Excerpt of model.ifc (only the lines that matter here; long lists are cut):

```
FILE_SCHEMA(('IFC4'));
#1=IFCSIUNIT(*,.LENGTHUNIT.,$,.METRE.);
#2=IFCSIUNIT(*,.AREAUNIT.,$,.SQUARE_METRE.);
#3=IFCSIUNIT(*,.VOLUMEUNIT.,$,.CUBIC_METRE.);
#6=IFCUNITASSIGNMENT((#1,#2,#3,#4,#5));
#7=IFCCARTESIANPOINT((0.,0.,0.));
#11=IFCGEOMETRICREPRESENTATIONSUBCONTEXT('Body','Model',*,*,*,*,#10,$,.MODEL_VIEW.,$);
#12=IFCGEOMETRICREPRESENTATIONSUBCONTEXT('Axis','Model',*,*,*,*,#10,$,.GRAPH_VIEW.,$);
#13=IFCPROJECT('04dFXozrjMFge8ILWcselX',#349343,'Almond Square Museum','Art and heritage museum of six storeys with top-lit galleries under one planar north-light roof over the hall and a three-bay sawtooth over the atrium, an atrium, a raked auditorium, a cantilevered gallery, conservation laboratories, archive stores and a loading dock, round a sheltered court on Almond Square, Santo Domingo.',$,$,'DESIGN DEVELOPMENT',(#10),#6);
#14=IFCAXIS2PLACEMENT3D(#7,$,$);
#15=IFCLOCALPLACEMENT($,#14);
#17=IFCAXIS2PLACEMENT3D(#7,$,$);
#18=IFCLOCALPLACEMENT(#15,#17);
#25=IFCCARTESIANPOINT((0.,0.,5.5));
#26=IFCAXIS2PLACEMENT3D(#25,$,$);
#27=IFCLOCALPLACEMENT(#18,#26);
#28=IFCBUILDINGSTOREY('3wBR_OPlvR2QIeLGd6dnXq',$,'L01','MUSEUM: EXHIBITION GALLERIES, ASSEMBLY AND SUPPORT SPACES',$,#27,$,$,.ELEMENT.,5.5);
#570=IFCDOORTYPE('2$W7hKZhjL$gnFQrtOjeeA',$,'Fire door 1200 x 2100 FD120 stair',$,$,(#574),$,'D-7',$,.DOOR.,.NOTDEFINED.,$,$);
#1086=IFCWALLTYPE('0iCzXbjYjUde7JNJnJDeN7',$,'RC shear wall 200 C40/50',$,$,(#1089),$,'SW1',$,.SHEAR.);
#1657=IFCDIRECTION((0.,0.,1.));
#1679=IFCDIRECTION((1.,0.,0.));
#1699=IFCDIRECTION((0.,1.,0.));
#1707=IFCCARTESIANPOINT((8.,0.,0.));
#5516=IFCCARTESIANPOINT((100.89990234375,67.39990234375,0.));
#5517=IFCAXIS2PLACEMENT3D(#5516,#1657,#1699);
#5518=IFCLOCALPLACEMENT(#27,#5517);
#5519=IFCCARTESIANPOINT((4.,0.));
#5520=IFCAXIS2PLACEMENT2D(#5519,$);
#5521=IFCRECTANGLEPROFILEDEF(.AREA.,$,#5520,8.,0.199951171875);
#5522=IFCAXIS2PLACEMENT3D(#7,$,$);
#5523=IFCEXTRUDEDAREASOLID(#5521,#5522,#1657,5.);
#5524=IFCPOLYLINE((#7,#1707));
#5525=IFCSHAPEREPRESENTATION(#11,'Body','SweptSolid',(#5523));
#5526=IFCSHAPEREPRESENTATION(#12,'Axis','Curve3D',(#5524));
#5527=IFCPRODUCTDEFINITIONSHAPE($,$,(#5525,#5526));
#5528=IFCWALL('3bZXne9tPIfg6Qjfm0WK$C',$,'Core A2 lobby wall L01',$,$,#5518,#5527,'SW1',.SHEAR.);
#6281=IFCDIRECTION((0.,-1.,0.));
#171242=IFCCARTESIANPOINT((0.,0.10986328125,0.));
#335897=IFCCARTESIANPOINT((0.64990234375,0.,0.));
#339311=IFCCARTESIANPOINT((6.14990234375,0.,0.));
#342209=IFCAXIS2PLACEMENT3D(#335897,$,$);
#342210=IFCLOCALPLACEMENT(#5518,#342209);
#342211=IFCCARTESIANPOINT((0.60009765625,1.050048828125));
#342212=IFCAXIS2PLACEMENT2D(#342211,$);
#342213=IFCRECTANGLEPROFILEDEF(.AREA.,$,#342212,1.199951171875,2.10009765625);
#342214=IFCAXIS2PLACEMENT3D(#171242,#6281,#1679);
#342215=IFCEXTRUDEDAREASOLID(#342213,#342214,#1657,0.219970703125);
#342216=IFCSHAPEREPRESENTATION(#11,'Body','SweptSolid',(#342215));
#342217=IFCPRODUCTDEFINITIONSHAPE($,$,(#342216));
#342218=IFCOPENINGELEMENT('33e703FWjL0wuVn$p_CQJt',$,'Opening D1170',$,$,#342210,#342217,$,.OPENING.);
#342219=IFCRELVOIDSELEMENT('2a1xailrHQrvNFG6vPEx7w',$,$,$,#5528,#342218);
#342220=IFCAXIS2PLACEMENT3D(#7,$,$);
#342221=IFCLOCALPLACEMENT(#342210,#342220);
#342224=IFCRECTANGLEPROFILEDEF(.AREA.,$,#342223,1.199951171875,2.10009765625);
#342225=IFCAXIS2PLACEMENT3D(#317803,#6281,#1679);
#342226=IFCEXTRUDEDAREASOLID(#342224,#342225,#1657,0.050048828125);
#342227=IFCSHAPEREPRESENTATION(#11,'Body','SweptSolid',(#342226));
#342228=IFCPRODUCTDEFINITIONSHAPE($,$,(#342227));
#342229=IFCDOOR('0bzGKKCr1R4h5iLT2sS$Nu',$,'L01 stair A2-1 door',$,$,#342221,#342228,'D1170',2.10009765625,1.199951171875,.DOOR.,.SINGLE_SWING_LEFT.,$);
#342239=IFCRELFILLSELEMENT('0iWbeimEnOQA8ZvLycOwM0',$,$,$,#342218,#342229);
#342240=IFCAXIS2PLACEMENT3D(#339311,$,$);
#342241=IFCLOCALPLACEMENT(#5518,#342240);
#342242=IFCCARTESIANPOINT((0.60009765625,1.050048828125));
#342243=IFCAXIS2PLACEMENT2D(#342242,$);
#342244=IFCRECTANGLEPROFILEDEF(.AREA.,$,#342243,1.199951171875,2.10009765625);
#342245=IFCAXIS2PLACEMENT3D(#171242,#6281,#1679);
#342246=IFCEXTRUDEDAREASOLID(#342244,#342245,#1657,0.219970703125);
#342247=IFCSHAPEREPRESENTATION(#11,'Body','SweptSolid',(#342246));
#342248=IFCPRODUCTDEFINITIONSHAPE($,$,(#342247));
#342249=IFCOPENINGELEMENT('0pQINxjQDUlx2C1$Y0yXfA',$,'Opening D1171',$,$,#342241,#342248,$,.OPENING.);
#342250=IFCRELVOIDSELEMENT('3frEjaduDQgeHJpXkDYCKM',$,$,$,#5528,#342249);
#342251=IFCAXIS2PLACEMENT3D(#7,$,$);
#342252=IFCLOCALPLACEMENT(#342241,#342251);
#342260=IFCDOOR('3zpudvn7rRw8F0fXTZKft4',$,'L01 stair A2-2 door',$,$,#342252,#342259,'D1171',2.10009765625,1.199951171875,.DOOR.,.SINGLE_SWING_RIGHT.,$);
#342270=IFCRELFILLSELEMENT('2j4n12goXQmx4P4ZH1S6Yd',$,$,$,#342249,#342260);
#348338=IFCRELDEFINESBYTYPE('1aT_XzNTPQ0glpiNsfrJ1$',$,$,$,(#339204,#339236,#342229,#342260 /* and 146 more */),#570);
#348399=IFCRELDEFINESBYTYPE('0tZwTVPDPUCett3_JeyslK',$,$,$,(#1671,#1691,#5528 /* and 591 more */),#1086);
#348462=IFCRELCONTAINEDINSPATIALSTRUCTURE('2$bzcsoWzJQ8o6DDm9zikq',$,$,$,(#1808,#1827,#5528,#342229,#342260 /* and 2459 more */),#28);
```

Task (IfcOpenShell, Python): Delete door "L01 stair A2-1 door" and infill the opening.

```python
import ifcopenshell
import ifcopenshell.api.feature
import ifcopenshell.api.root
import ifcopenshell.geom
import ifcopenshell.util.shape

model = ifcopenshell.open("model.ifc")
settings = ifcopenshell.geom.settings()


def volume(element):
    """Net volume in cubic metres, openings subtracted."""
    shape = ifcopenshell.geom.create_shape(settings, element)
    return ifcopenshell.util.shape.get_volume(shape.geometry)


door = model.by_guid("0bzGKKCr1R4h5iLT2sS$Nu")
opening = door.FillsVoids[0].RelatingOpeningElement
wall = opening.VoidsElements[0].RelatingBuildingElement
before = volume(wall)

ifcopenshell.api.root.remove_product(model, product=door)
ifcopenshell.api.feature.remove_feature(model, feature=opening)

after = volume(wall)

print(f"wall volume {before:.3f} -> {after:.3f} m3")

model.write("model_updated.ifc")
```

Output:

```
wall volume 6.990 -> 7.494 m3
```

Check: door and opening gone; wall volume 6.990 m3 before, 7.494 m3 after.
